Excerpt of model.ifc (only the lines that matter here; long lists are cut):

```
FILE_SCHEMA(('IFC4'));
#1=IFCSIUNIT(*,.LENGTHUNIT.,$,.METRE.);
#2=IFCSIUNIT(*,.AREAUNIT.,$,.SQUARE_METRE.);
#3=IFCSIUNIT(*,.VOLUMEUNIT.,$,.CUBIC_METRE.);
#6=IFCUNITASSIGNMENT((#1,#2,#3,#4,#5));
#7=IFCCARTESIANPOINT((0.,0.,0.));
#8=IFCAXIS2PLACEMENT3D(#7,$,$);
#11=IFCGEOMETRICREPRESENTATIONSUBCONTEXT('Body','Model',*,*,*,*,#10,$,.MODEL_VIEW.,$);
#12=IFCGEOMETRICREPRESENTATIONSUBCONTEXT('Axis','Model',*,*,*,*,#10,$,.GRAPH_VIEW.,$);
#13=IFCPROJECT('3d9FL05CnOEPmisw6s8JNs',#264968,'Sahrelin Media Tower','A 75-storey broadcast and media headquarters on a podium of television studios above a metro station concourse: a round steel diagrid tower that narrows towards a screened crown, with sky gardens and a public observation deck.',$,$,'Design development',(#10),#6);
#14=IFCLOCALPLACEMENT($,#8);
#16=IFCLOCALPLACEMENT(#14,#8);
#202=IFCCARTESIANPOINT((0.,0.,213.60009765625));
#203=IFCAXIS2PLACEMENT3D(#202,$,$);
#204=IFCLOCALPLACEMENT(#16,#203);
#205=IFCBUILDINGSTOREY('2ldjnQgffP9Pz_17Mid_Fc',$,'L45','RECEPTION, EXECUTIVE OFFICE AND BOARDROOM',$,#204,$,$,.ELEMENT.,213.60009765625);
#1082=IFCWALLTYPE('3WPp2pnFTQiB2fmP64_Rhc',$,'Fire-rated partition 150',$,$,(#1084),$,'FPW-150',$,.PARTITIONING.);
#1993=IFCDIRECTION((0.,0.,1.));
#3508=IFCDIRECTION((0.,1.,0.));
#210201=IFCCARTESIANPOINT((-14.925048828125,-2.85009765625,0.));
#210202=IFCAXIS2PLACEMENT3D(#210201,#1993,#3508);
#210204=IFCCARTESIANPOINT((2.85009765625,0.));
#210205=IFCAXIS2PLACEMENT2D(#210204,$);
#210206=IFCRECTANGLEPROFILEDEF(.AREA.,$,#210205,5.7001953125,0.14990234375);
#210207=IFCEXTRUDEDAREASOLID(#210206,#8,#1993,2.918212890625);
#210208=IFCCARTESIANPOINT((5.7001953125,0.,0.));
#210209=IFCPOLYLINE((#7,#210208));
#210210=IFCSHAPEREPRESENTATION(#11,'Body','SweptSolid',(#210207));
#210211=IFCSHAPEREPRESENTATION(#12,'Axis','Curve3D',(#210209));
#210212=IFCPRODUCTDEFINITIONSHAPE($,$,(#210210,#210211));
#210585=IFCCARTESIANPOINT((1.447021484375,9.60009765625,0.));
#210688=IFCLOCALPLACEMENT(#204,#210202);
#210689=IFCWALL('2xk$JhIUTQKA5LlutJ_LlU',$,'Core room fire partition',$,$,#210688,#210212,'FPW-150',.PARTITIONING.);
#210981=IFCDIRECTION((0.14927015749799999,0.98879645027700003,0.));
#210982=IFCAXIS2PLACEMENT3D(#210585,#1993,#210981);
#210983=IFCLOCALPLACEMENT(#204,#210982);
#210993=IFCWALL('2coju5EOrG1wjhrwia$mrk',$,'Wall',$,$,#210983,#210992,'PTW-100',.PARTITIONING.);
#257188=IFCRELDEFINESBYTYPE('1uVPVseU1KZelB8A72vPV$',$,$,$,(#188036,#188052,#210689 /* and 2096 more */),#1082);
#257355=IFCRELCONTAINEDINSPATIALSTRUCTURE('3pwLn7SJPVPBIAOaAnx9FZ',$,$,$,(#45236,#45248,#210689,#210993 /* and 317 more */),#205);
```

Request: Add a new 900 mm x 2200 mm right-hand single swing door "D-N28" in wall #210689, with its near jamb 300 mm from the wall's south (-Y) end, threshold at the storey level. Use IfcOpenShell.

```python
import numpy as np
import ifcopenshell
import ifcopenshell.api.feature
import ifcopenshell.api.geometry
import ifcopenshell.api.root
import ifcopenshell.api.spatial
import ifcopenshell.geom
import ifcopenshell.util.element
import ifcopenshell.util.placement
import ifcopenshell.util.representation
import ifcopenshell.util.shape
import ifcopenshell.util.unit

model = ifcopenshell.open("model.ifc")
unit_scale = ifcopenshell.util.unit.calculate_unit_scale(model)
settings = ifcopenshell.geom.settings()


def volume(element):
    """Net volume in cubic metres, openings subtracted."""
    shape = ifcopenshell.geom.create_shape(settings, element)
    return ifcopenshell.util.shape.get_volume(shape.geometry)


wall = model.by_guid("2xk$JhIUTQKA5LlutJ_LlU")
storey = ifcopenshell.util.element.get_container(wall, ifc_class="IfcBuildingStorey")
context = ifcopenshell.util.representation.get_context(model, "Model", "Body", "MODEL_VIEW")
before = volume(wall)

width, height, from_end, sill = 0.9, 2.2, 0.3, 0.0  # metres

# The wall runs along its own X axis, and the end named is its -X end.
wall_shape = ifcopenshell.geom.create_shape(settings, wall)
x, y, z = ifcopenshell.util.shape.get_vertices(wall_shape.geometry).T
start = x.min() + from_end
face, thickness = float(y.min()), float(y.max() - y.min())
wall_matrix = ifcopenshell.util.placement.get_local_placement(wall.ObjectPlacement)
level = ifcopenshell.util.placement.get_local_placement(storey.ObjectPlacement)[2, 3]


def in_wall(x, y):
    """Placement at x, y metres in the wall's axes, at sill height."""
    matrix = wall_matrix.copy()
    matrix[:, 3] = wall_matrix @ np.array([x / unit_scale, y / unit_scale, 0.0, 1.0])
    matrix[2, 3] = level + sill / unit_scale
    return matrix


# Opening: a box that overshoots both wall faces by 50 mm.
opening = ifcopenshell.api.root.create_entity(model, ifc_class="IfcOpeningElement", predefined_type="OPENING")
box = ifcopenshell.api.geometry.add_wall_representation(
    model, context=context, length=width, height=height, thickness=thickness + 0.1
)
ifcopenshell.api.geometry.assign_representation(model, product=opening, representation=box)
ifcopenshell.api.geometry.edit_object_placement(model, product=opening, matrix=in_wall(start, face - 0.05), is_si=False)
ifcopenshell.api.feature.add_feature(model, feature=opening, element=wall)

door = ifcopenshell.api.root.create_entity(model, ifc_class="IfcDoor", name="D-N28", predefined_type="DOOR")
door.OverallWidth, door.OverallHeight = width / unit_scale, height / unit_scale
door.OperationType = "SINGLE_SWING_RIGHT"
body = ifcopenshell.api.geometry.add_door_representation(
    model,
    context=context,
    overall_width=door.OverallWidth,
    overall_height=door.OverallHeight,
    operation_type="SINGLE_SWING_RIGHT",
    lining_properties={"LiningDepth": thickness / unit_scale, "ThresholdDepth": thickness / unit_scale},
)
ifcopenshell.api.geometry.assign_representation(model, product=door, representation=body)
ifcopenshell.api.spatial.assign_container(model, products=[door], relating_structure=storey)
ifcopenshell.api.feature.add_filling(model, opening=opening, element=door)

# The lining spans the wall, so the door starts at the wall face.
ifcopenshell.api.geometry.edit_object_placement(model, product=door, matrix=in_wall(start, face), is_si=False)

after = volume(wall)

print(f"wall volume {before:.3f} -> {after:.3f} m3")

model.write("model_updated.ifc")
```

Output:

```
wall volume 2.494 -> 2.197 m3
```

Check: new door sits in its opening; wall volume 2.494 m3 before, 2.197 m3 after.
